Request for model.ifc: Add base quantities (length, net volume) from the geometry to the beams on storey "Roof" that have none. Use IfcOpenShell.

First a look at what the model holds.

```python
import ifcopenshell
import ifcopenshell.util.element
import ifcopenshell.util.unit

model = ifcopenshell.open("model.ifc")
print(model.schema)
for unit_type in ("LENGTHUNIT", "AREAUNIT", "VOLUMEUNIT"):
    print(unit_type, ifcopenshell.util.unit.calculate_unit_scale(model, unit_type))
storey = next(s for s in model.by_type("IfcBuildingStorey") if s.Name == "Roof")
beams = [e for e in ifcopenshell.util.element.get_decomposition(storey) if e.is_a("IfcBeam")]
for e in sorted(beams, key=lambda e: e.id()):
    print(e.id(), e.is_a(), e.Name, list(ifcopenshell.util.element.get_psets(e, qtos_only=True)), sep=" | ")
```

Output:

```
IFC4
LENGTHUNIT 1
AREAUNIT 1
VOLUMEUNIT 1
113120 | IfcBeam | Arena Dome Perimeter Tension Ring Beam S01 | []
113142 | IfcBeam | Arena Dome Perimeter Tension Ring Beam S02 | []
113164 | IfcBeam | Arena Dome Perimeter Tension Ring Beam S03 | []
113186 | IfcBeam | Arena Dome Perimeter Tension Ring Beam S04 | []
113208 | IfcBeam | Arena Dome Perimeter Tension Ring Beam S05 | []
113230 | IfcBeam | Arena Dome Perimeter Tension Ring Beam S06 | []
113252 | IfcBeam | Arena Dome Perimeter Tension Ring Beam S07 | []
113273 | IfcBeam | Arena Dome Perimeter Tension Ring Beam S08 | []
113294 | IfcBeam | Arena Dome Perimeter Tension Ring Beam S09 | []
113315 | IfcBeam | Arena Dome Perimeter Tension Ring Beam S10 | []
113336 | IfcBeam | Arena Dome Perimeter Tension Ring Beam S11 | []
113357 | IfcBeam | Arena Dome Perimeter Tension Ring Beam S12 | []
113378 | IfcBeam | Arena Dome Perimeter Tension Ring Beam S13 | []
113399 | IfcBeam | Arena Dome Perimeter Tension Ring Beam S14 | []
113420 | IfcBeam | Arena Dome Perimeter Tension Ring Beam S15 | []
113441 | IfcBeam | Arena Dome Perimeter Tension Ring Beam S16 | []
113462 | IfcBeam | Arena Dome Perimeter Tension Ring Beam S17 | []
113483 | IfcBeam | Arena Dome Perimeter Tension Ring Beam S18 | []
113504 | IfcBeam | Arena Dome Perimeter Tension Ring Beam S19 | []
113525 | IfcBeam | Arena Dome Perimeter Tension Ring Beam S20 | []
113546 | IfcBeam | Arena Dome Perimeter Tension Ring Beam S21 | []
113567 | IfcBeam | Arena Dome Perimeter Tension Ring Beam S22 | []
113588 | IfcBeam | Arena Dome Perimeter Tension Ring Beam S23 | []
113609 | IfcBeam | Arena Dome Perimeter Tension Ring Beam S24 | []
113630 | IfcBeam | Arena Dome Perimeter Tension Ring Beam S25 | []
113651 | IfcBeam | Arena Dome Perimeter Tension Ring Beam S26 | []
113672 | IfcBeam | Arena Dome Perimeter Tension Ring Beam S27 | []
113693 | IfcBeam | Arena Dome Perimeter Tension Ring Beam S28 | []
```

```python
import ifcopenshell
import ifcopenshell.api.pset
import ifcopenshell.geom
import ifcopenshell.util.element
import ifcopenshell.util.shape
import ifcopenshell.util.unit

model = ifcopenshell.open("model.ifc")
unit_scale = ifcopenshell.util.unit.calculate_unit_scale(model)
volume_scale = ifcopenshell.util.unit.calculate_unit_scale(model, "VOLUMEUNIT")
settings = ifcopenshell.geom.settings()

storey = next(s for s in model.by_type("IfcBuildingStorey") if s.Name == "Roof")
beams = [e for e in ifcopenshell.util.element.get_decomposition(storey) if e.is_a("IfcBeam")]

for e in sorted(beams, key=lambda e: e.id()):
    if ifcopenshell.util.element.get_psets(e, qtos_only=True, should_inherit=False):
        continue
    # Geometry comes back in metres, in the element's own axes.
    shape = ifcopenshell.geom.create_shape(settings, e)
    values = {
        "Length": ifcopenshell.util.shape.get_max_xyz(shape.geometry) / unit_scale,
        "NetVolume": ifcopenshell.util.shape.get_volume(shape.geometry) / volume_scale,
    }
    qto = ifcopenshell.api.pset.add_qto(model, product=e, name="Qto_BeamBaseQuantities")
    ifcopenshell.api.pset.edit_qto(model, qto=qto, properties=values)
    print(e.id(), {k: round(v, 3) for k, v in values.items()})

model.write("model_edited.ifc")
```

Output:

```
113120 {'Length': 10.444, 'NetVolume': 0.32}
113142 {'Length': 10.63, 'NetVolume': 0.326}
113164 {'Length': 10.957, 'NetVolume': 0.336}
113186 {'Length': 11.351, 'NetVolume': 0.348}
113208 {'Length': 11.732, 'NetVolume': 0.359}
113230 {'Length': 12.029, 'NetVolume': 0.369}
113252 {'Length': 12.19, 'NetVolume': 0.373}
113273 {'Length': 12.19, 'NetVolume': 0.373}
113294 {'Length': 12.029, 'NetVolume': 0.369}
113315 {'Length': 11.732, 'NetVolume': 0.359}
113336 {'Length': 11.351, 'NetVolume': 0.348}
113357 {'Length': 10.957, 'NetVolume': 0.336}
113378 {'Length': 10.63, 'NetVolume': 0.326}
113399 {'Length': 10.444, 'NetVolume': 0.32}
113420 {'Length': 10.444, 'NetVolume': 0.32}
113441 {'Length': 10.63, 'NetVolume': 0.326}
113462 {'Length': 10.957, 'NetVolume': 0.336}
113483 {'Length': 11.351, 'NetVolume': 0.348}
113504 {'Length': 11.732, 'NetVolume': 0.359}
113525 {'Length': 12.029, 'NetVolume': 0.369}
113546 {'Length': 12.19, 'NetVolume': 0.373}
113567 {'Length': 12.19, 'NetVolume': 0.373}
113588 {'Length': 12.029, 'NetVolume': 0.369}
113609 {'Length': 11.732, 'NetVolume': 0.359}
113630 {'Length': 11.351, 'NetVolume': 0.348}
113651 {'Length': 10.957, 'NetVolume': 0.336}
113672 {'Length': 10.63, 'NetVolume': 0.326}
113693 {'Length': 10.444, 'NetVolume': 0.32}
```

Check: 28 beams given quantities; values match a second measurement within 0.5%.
